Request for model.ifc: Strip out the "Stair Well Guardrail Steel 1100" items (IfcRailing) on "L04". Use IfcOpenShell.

First a look at what the model holds.

```python
import ifcopenshell
import ifcopenshell.util.element

model = ifcopenshell.open("model.ifc")
print(model.schema)
storey = next(s for s in model.by_type("IfcBuildingStorey") if s.Name == "L04")
railings = [e for e in ifcopenshell.util.element.get_decomposition(storey) if e.is_a("IfcRailing")]
seen = {}
for e in railings:
    element_type = ifcopenshell.util.element.get_type(e)
    name = element_type.Name if element_type not in (None, e) else None
    seen[name] = seen.get(name, 0) + 1
for name, count in sorted(seen.items(), key=str):
    print(count, "x", name)
```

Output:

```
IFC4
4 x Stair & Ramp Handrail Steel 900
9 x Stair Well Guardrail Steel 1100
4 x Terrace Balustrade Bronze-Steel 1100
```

```python
import ifcopenshell
import ifcopenshell.api.root
import ifcopenshell.util.element

model = ifcopenshell.open("model.ifc")

storey = next(s for s in model.by_type("IfcBuildingStorey") if s.Name == "L04")
railings = [e for e in ifcopenshell.util.element.get_decomposition(storey) if e.is_a("IfcRailing")]
targets = [e for e in railings if (t := ifcopenshell.util.element.get_type(e)) not in (None, e) and t.Name == "Stair Well Guardrail Steel 1100"]

for e in targets:
    ifcopenshell.api.root.remove_product(model, product=e)
print(len(targets), "removed")

model.write("model-out.ifc")
```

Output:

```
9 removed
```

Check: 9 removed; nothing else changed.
